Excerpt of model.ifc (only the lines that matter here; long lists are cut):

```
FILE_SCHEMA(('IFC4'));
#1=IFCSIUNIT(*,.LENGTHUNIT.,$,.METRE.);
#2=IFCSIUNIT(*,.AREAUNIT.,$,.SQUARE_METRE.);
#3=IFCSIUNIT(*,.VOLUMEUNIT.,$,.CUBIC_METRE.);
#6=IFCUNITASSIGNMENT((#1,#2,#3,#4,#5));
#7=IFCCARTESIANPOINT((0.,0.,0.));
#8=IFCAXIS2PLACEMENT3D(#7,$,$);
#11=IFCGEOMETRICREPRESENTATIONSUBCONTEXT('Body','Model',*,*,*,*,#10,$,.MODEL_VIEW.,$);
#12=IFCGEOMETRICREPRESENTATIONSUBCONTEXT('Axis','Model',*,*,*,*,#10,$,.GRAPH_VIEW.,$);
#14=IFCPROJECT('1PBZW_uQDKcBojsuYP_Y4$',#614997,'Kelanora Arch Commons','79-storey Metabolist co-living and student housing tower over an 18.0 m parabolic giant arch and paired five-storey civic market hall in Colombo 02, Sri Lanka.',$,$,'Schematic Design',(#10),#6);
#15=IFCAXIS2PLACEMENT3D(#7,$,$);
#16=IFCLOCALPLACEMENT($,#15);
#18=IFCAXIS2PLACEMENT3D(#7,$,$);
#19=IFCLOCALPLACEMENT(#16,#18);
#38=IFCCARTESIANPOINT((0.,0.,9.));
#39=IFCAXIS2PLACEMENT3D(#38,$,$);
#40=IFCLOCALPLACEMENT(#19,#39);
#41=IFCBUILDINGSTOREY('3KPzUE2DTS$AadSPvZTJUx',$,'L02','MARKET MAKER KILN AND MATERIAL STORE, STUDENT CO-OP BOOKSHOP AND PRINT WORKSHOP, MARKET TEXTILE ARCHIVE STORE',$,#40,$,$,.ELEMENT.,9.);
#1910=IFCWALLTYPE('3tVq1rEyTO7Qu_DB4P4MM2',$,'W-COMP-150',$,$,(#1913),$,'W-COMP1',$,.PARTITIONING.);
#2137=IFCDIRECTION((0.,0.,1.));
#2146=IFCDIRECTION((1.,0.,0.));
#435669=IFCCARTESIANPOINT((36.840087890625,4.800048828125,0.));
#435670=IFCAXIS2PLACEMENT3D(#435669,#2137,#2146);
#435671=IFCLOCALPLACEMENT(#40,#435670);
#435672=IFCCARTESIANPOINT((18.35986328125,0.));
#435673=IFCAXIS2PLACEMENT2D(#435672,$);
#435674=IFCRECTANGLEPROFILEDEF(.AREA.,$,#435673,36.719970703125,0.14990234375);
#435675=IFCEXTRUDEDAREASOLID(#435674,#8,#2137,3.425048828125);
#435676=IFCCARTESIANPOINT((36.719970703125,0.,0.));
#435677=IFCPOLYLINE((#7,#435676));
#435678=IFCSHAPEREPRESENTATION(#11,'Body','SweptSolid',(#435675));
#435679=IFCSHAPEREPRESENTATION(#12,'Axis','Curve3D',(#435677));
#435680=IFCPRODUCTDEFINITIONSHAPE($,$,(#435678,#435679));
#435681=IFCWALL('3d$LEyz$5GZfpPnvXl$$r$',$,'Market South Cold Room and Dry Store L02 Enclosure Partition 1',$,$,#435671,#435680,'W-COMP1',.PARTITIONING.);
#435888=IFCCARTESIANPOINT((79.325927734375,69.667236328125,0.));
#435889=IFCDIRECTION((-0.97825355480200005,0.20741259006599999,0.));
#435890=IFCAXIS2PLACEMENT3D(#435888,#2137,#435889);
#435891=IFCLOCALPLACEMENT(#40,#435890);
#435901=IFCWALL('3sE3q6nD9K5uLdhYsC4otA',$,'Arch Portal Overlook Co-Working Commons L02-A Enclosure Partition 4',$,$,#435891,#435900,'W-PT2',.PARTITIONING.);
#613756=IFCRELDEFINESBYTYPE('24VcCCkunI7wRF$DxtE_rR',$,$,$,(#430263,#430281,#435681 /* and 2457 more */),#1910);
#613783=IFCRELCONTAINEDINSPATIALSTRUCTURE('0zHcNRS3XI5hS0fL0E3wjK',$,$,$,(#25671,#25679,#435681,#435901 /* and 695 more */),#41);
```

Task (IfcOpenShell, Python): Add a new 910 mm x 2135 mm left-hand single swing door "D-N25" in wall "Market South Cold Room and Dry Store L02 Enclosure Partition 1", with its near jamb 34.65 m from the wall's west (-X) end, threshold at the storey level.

```python
import numpy as np
import ifcopenshell
import ifcopenshell.api.feature
import ifcopenshell.api.geometry
import ifcopenshell.api.root
import ifcopenshell.api.spatial
import ifcopenshell.geom
import ifcopenshell.util.element
import ifcopenshell.util.placement
import ifcopenshell.util.representation
import ifcopenshell.util.shape
import ifcopenshell.util.unit

model = ifcopenshell.open("model.ifc")
unit_scale = ifcopenshell.util.unit.calculate_unit_scale(model)
settings = ifcopenshell.geom.settings()


def volume(element):
    """Net volume in cubic metres, openings subtracted."""
    shape = ifcopenshell.geom.create_shape(settings, element)
    return ifcopenshell.util.shape.get_volume(shape.geometry)


wall = model.by_guid("3d$LEyz$5GZfpPnvXl$$r$")
storey = ifcopenshell.util.element.get_container(wall, ifc_class="IfcBuildingStorey")
context = ifcopenshell.util.representation.get_context(model, "Model", "Body", "MODEL_VIEW")
before = volume(wall)

width, height, from_end, sill = 0.91, 2.135, 34.65, 0.0  # metres

# The wall runs along its own X axis, and the end named is its -X end.
wall_shape = ifcopenshell.geom.create_shape(settings, wall)
x, y, z = ifcopenshell.util.shape.get_vertices(wall_shape.geometry).T
start = x.min() + from_end
face, thickness = float(y.min()), float(y.max() - y.min())
wall_matrix = ifcopenshell.util.placement.get_local_placement(wall.ObjectPlacement)
level = ifcopenshell.util.placement.get_local_placement(storey.ObjectPlacement)[2, 3]


def in_wall(x, y):
    """Placement at x, y metres in the wall's axes, at sill height."""
    matrix = wall_matrix.copy()
    matrix[:, 3] = wall_matrix @ np.array([x / unit_scale, y / unit_scale, 0.0, 1.0])
    matrix[2, 3] = level + sill / unit_scale
    return matrix


# Opening: a box that overshoots both wall faces by 50 mm.
opening = ifcopenshell.api.root.create_entity(model, ifc_class="IfcOpeningElement", predefined_type="OPENING")
box = ifcopenshell.api.geometry.add_wall_representation(
    model, context=context, length=width, height=height, thickness=thickness + 0.1
)
ifcopenshell.api.geometry.assign_representation(model, product=opening, representation=box)
ifcopenshell.api.geometry.edit_object_placement(model, product=opening, matrix=in_wall(start, face - 0.05), is_si=False)
ifcopenshell.api.feature.add_feature(model, feature=opening, element=wall)

door = ifcopenshell.api.root.create_entity(model, ifc_class="IfcDoor", name="D-N25", predefined_type="DOOR")
door.OverallWidth, door.OverallHeight = width / unit_scale, height / unit_scale
door.OperationType = "SINGLE_SWING_LEFT"
body = ifcopenshell.api.geometry.add_door_representation(
    model,
    context=context,
    overall_width=door.OverallWidth,
    overall_height=door.OverallHeight,
    operation_type="SINGLE_SWING_LEFT",
    lining_properties={"LiningDepth": thickness / unit_scale, "ThresholdDepth": thickness / unit_scale},
)
ifcopenshell.api.geometry.assign_representation(model, product=door, representation=body)
ifcopenshell.api.spatial.assign_container(model, products=[door], relating_structure=storey)
ifcopenshell.api.feature.add_filling(model, opening=opening, element=door)

# The lining spans the wall, so the door starts at the wall face.
ifcopenshell.api.geometry.edit_object_placement(model, product=door, matrix=in_wall(start, face), is_si=False)

after = volume(wall)

print(f"wall volume {before:.3f} -> {after:.3f} m3")

model.write("model_v2.ifc")
```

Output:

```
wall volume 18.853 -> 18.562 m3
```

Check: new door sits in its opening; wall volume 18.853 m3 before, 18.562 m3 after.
